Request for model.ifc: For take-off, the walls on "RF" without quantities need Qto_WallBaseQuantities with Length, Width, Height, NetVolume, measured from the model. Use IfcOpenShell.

First a look at what the model holds.

```python
import ifcopenshell
import ifcopenshell.util.element
import ifcopenshell.util.unit

model = ifcopenshell.open("model.ifc")
print(model.schema)
for unit_type in ("LENGTHUNIT", "AREAUNIT", "VOLUMEUNIT"):
    print(unit_type, ifcopenshell.util.unit.calculate_unit_scale(model, unit_type))
storey = next(s for s in model.by_type("IfcBuildingStorey") if s.Name == "RF")
walls = [e for e in ifcopenshell.util.element.get_decomposition(storey) if e.is_a("IfcWall")]
for e in sorted(walls, key=lambda e: e.id()):
    print(e.id(), e.is_a(), e.Name, list(ifcopenshell.util.element.get_psets(e, qtos_only=True)), sep=" | ")
```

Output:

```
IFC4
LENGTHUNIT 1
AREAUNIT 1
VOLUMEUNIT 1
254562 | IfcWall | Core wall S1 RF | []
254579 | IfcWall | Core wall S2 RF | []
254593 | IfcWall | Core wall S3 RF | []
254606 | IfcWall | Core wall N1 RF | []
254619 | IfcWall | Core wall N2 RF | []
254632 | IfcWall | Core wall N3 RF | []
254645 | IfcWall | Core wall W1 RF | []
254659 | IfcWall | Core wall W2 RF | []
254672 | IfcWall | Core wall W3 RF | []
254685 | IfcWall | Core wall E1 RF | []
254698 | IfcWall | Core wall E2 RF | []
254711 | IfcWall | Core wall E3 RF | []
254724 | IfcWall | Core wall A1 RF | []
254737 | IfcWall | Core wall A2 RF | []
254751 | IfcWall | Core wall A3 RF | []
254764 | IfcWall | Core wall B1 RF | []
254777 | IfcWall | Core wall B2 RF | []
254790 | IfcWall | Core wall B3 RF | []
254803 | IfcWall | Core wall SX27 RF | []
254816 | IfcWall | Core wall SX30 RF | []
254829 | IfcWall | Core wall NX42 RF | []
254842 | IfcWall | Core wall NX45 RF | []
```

```python
import ifcopenshell
import ifcopenshell.api.pset
import ifcopenshell.geom
import ifcopenshell.util.element
import ifcopenshell.util.shape
import ifcopenshell.util.unit

model = ifcopenshell.open("model.ifc")
unit_scale = ifcopenshell.util.unit.calculate_unit_scale(model)
volume_scale = ifcopenshell.util.unit.calculate_unit_scale(model, "VOLUMEUNIT")
settings = ifcopenshell.geom.settings()

storey = next(s for s in model.by_type("IfcBuildingStorey") if s.Name == "RF")
walls = [e for e in ifcopenshell.util.element.get_decomposition(storey) if e.is_a("IfcWall")]

for e in sorted(walls, key=lambda e: e.id()):
    if ifcopenshell.util.element.get_psets(e, qtos_only=True, should_inherit=False):
        continue
    # Geometry comes back in metres, in the element's own axes.
    shape = ifcopenshell.geom.create_shape(settings, e)
    values = {
        "Length": ifcopenshell.util.shape.get_x(shape.geometry) / unit_scale,
        "Width": ifcopenshell.util.shape.get_y(shape.geometry) / unit_scale,
        "Height": ifcopenshell.util.shape.get_z(shape.geometry) / unit_scale,
        "NetVolume": ifcopenshell.util.shape.get_volume(shape.geometry) / volume_scale,
    }
    qto = ifcopenshell.api.pset.add_qto(model, product=e, name="Qto_WallBaseQuantities")
    ifcopenshell.api.pset.edit_qto(model, qto=qto, properties=values)
    print(e.id(), {k: round(v, 3) for k, v in values.items()})

model.write("model_updated.ifc")
```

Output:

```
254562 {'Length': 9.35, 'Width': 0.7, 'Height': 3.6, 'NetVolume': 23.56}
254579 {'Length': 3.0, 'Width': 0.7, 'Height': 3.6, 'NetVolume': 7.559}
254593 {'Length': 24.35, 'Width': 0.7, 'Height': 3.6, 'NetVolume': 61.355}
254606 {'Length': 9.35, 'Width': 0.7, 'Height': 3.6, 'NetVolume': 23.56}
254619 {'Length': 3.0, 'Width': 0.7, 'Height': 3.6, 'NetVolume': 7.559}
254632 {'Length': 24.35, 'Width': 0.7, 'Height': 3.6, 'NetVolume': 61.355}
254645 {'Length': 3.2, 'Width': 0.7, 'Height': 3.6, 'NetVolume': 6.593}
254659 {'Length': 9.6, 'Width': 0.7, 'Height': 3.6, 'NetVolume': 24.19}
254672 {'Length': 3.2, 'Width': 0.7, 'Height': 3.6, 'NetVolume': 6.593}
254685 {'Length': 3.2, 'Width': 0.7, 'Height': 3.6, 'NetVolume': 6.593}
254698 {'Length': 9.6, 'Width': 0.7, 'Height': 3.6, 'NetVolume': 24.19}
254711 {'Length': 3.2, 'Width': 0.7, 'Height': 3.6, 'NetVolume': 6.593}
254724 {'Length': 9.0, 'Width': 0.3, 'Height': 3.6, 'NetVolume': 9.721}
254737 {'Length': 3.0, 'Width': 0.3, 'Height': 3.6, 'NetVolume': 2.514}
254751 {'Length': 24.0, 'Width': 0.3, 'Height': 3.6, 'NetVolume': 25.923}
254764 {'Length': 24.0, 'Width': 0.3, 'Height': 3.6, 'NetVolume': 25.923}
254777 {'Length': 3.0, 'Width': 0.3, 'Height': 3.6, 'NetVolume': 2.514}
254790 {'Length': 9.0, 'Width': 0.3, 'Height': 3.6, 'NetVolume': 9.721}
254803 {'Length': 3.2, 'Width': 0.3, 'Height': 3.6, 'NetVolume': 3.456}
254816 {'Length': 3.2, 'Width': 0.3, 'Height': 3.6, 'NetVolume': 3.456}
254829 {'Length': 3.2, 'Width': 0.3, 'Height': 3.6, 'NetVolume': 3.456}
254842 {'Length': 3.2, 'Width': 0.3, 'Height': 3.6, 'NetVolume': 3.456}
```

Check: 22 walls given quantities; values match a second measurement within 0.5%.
